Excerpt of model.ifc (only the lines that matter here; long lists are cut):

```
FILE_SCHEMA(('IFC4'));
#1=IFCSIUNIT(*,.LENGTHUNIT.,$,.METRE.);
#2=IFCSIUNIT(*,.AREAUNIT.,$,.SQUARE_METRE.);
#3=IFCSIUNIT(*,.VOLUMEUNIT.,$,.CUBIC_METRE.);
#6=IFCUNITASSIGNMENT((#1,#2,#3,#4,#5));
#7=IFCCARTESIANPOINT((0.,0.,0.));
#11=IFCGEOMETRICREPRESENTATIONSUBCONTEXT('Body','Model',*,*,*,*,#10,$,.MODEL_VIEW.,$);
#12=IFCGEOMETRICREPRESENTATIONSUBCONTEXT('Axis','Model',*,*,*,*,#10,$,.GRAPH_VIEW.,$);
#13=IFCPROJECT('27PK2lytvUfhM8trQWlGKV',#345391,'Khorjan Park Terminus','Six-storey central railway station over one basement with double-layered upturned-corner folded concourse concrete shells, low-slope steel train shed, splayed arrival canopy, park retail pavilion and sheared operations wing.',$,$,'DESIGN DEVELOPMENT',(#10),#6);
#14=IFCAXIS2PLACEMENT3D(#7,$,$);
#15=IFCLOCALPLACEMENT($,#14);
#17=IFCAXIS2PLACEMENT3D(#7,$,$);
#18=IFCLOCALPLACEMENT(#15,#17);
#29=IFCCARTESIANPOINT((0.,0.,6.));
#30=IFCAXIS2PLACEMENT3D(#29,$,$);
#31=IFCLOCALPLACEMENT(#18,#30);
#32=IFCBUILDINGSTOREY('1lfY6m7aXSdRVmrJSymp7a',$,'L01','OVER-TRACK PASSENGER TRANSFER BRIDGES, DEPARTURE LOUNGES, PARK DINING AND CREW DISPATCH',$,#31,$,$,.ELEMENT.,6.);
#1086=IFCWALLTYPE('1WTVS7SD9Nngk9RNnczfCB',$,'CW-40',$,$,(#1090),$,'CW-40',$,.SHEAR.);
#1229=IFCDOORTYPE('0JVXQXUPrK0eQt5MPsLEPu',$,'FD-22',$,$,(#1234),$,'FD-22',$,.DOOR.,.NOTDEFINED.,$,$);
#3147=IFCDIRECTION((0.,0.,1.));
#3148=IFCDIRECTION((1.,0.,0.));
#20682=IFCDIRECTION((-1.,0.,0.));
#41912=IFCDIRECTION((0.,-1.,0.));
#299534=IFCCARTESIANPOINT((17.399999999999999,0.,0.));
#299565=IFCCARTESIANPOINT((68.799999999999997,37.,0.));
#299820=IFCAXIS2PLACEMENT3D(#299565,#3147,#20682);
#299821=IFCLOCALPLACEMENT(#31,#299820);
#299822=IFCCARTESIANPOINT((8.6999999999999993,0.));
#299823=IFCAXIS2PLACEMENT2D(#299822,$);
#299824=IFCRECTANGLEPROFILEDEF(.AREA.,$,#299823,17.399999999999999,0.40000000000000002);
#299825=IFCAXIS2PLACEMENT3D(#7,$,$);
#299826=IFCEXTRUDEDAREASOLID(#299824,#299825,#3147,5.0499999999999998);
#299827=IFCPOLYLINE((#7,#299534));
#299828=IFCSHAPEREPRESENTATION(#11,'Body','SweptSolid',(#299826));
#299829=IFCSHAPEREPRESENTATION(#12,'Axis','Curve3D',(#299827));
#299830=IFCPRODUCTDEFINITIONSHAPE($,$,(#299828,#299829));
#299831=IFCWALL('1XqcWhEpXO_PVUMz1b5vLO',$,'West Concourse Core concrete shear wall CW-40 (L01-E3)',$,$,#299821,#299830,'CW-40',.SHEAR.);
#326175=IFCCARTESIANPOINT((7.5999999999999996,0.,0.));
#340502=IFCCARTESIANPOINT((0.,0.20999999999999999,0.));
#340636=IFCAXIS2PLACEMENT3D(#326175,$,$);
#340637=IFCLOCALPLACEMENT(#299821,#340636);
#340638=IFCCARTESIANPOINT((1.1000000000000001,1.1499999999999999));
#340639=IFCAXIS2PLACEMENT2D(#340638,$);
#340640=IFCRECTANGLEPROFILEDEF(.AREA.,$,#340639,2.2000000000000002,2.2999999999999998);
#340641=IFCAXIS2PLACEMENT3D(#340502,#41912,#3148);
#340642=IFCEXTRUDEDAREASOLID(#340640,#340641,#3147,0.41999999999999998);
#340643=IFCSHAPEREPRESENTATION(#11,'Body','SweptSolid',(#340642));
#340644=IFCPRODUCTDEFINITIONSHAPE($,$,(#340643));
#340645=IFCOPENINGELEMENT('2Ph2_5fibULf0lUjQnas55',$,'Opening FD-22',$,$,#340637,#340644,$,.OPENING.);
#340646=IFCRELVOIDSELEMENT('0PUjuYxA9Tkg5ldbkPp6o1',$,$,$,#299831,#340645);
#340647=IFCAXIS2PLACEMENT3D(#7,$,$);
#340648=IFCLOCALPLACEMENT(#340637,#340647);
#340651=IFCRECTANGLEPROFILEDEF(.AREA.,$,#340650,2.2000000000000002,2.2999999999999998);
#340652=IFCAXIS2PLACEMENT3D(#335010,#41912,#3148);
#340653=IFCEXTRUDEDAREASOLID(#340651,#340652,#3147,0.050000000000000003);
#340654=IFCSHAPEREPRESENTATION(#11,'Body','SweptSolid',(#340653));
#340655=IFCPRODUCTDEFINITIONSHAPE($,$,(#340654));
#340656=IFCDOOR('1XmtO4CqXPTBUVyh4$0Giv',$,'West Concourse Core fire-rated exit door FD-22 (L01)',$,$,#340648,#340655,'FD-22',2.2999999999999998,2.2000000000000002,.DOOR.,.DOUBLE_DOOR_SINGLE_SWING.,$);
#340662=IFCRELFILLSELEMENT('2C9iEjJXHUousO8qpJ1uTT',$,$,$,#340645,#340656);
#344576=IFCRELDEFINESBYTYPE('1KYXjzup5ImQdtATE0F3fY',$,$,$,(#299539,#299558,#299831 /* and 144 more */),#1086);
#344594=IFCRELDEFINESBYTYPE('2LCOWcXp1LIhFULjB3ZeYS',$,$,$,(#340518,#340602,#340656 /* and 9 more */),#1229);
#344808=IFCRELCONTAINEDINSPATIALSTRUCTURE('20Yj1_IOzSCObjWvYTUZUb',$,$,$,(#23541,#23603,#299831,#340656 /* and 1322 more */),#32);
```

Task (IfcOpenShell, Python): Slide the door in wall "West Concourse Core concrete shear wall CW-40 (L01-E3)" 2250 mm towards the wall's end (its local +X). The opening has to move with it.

```python
import ifcopenshell
import ifcopenshell.api.geometry
import ifcopenshell.util.placement
import ifcopenshell.util.unit

model = ifcopenshell.open("model.ifc")
unit_scale = ifcopenshell.util.unit.calculate_unit_scale(model)

door = model.by_guid("1XmtO4CqXPTBUVyh4$0Giv")
opening = door.FillsVoids[0].RelatingOpeningElement
wall = opening.VoidsElements[0].RelatingBuildingElement

wall_matrix = ifcopenshell.util.placement.get_local_placement(wall.ObjectPlacement)
shift = wall_matrix[:3, 0] * 2.25 / unit_scale
before = ifcopenshell.util.placement.get_local_placement(door.ObjectPlacement)[:3, 3].copy()

# The door is placed relative to its opening, so it follows when the opening moves.
matrix = ifcopenshell.util.placement.get_local_placement(opening.ObjectPlacement)
matrix[:3, 3] += shift
ifcopenshell.api.geometry.edit_object_placement(
    model, product=opening, matrix=matrix, is_si=False, should_transform_children=True
)

after = ifcopenshell.util.placement.get_local_placement(door.ObjectPlacement)[:3, 3]
print("door moved by", (after - before).round(3) + 0.0)

model.write("model_edited.ifc")
```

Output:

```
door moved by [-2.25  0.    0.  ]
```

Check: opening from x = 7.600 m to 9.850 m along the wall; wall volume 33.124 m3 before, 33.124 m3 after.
